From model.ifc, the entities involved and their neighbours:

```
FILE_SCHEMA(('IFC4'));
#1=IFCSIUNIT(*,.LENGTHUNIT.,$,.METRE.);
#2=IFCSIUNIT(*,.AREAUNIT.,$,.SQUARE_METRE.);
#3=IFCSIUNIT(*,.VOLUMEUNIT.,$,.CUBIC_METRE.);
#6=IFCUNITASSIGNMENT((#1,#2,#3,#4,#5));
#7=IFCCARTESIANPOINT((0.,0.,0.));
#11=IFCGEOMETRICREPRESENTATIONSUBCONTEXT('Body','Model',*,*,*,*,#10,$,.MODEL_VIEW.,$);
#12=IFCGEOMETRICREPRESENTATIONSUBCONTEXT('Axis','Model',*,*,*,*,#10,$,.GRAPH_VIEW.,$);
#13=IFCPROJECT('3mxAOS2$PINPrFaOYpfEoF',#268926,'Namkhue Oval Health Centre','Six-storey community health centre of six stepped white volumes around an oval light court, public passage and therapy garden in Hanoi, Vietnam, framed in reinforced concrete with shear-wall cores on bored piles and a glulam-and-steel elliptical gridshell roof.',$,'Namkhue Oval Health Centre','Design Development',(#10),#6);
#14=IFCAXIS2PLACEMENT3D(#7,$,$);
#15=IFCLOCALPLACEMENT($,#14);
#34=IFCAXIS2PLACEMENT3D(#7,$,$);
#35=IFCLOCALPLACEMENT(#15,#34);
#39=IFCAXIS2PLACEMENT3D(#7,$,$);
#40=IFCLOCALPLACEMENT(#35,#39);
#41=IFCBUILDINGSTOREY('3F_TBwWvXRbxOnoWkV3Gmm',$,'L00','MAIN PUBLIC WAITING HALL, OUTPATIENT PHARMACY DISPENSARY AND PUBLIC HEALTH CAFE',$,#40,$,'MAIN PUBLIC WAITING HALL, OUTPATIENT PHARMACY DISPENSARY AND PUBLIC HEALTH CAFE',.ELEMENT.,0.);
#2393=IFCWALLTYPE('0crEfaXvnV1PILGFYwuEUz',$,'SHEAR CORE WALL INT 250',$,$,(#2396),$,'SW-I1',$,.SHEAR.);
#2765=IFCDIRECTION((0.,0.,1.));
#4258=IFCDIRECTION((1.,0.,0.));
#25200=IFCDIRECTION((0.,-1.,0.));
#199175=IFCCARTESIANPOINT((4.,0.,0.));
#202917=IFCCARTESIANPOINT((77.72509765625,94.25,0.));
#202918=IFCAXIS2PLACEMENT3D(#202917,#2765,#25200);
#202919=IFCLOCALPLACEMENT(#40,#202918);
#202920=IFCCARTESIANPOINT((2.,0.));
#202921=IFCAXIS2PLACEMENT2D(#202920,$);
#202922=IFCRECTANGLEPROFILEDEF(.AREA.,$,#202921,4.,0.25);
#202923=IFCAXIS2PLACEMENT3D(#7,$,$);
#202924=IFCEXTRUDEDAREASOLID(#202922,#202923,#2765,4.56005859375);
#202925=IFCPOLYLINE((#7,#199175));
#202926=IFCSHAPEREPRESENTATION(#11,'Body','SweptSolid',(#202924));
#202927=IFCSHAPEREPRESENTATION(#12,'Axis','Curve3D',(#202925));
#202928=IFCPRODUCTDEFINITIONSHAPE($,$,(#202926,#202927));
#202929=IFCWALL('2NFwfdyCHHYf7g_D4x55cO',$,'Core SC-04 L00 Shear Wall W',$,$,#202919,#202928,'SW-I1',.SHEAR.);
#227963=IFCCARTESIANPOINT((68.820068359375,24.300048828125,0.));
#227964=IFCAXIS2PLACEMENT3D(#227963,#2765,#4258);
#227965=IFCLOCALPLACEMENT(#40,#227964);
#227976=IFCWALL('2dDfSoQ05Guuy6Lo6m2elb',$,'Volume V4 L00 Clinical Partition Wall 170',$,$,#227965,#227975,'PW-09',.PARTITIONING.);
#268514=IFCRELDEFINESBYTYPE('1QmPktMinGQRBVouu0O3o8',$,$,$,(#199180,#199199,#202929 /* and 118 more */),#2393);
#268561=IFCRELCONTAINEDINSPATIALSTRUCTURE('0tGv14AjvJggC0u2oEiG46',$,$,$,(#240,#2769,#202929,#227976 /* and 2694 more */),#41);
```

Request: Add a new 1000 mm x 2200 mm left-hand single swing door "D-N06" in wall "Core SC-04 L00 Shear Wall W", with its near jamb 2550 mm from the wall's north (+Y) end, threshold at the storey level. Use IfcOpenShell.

```python
import numpy as np
import ifcopenshell
import ifcopenshell.api.feature
import ifcopenshell.api.geometry
import ifcopenshell.api.root
import ifcopenshell.api.spatial
import ifcopenshell.geom
import ifcopenshell.util.element
import ifcopenshell.util.placement
import ifcopenshell.util.representation
import ifcopenshell.util.shape
import ifcopenshell.util.unit

model = ifcopenshell.open("model.ifc")
unit_scale = ifcopenshell.util.unit.calculate_unit_scale(model)
settings = ifcopenshell.geom.settings()


def volume(element):
    """Net volume in cubic metres, openings subtracted."""
    shape = ifcopenshell.geom.create_shape(settings, element)
    return ifcopenshell.util.shape.get_volume(shape.geometry)


wall = model.by_id(202929)
storey = ifcopenshell.util.element.get_container(wall, ifc_class="IfcBuildingStorey")
context = ifcopenshell.util.representation.get_context(model, "Model", "Body", "MODEL_VIEW")
before = volume(wall)

width, height, from_end, sill = 1, 2.2, 2.55, 0.0  # metres

# The wall runs along its own X axis, and the end named is its -X end.
wall_shape = ifcopenshell.geom.create_shape(settings, wall)
x, y, z = ifcopenshell.util.shape.get_vertices(wall_shape.geometry).T
start = x.min() + from_end
face, thickness = float(y.min()), float(y.max() - y.min())
wall_matrix = ifcopenshell.util.placement.get_local_placement(wall.ObjectPlacement)
level = ifcopenshell.util.placement.get_local_placement(storey.ObjectPlacement)[2, 3]


def in_wall(x, y):
    """Placement at x, y metres in the wall's axes, at sill height."""
    matrix = wall_matrix.copy()
    matrix[:, 3] = wall_matrix @ np.array([x / unit_scale, y / unit_scale, 0.0, 1.0])
    matrix[2, 3] = level + sill / unit_scale
    return matrix


# Opening: a box that overshoots both wall faces by 50 mm.
opening = ifcopenshell.api.root.create_entity(model, ifc_class="IfcOpeningElement", predefined_type="OPENING")
box = ifcopenshell.api.geometry.add_wall_representation(
    model, context=context, length=width, height=height, thickness=thickness + 0.1
)
ifcopenshell.api.geometry.assign_representation(model, product=opening, representation=box)
ifcopenshell.api.geometry.edit_object_placement(model, product=opening, matrix=in_wall(start, face - 0.05), is_si=False)
ifcopenshell.api.feature.add_feature(model, feature=opening, element=wall)

door = ifcopenshell.api.root.create_entity(model, ifc_class="IfcDoor", name="D-N06", predefined_type="DOOR")
door.OverallWidth, door.OverallHeight = width / unit_scale, height / unit_scale
door.OperationType = "SINGLE_SWING_LEFT"
body = ifcopenshell.api.geometry.add_door_representation(
    model,
    context=context,
    overall_width=door.OverallWidth,
    overall_height=door.OverallHeight,
    operation_type="SINGLE_SWING_LEFT",
    lining_properties={"LiningDepth": thickness / unit_scale, "ThresholdDepth": thickness / unit_scale},
)
ifcopenshell.api.geometry.assign_representation(model, product=door, representation=body)
ifcopenshell.api.spatial.assign_container(model, products=[door], relating_structure=storey)
ifcopenshell.api.feature.add_filling(model, opening=opening, element=door)

# The lining spans the wall, so the door starts at the wall face.
ifcopenshell.api.geometry.edit_object_placement(model, product=door, matrix=in_wall(start, face), is_si=False)

after = volume(wall)

print(f"wall volume {before:.3f} -> {after:.3f} m3")

model.write("model_updated.ifc")
```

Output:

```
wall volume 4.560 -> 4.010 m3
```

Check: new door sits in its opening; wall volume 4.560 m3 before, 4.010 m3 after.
